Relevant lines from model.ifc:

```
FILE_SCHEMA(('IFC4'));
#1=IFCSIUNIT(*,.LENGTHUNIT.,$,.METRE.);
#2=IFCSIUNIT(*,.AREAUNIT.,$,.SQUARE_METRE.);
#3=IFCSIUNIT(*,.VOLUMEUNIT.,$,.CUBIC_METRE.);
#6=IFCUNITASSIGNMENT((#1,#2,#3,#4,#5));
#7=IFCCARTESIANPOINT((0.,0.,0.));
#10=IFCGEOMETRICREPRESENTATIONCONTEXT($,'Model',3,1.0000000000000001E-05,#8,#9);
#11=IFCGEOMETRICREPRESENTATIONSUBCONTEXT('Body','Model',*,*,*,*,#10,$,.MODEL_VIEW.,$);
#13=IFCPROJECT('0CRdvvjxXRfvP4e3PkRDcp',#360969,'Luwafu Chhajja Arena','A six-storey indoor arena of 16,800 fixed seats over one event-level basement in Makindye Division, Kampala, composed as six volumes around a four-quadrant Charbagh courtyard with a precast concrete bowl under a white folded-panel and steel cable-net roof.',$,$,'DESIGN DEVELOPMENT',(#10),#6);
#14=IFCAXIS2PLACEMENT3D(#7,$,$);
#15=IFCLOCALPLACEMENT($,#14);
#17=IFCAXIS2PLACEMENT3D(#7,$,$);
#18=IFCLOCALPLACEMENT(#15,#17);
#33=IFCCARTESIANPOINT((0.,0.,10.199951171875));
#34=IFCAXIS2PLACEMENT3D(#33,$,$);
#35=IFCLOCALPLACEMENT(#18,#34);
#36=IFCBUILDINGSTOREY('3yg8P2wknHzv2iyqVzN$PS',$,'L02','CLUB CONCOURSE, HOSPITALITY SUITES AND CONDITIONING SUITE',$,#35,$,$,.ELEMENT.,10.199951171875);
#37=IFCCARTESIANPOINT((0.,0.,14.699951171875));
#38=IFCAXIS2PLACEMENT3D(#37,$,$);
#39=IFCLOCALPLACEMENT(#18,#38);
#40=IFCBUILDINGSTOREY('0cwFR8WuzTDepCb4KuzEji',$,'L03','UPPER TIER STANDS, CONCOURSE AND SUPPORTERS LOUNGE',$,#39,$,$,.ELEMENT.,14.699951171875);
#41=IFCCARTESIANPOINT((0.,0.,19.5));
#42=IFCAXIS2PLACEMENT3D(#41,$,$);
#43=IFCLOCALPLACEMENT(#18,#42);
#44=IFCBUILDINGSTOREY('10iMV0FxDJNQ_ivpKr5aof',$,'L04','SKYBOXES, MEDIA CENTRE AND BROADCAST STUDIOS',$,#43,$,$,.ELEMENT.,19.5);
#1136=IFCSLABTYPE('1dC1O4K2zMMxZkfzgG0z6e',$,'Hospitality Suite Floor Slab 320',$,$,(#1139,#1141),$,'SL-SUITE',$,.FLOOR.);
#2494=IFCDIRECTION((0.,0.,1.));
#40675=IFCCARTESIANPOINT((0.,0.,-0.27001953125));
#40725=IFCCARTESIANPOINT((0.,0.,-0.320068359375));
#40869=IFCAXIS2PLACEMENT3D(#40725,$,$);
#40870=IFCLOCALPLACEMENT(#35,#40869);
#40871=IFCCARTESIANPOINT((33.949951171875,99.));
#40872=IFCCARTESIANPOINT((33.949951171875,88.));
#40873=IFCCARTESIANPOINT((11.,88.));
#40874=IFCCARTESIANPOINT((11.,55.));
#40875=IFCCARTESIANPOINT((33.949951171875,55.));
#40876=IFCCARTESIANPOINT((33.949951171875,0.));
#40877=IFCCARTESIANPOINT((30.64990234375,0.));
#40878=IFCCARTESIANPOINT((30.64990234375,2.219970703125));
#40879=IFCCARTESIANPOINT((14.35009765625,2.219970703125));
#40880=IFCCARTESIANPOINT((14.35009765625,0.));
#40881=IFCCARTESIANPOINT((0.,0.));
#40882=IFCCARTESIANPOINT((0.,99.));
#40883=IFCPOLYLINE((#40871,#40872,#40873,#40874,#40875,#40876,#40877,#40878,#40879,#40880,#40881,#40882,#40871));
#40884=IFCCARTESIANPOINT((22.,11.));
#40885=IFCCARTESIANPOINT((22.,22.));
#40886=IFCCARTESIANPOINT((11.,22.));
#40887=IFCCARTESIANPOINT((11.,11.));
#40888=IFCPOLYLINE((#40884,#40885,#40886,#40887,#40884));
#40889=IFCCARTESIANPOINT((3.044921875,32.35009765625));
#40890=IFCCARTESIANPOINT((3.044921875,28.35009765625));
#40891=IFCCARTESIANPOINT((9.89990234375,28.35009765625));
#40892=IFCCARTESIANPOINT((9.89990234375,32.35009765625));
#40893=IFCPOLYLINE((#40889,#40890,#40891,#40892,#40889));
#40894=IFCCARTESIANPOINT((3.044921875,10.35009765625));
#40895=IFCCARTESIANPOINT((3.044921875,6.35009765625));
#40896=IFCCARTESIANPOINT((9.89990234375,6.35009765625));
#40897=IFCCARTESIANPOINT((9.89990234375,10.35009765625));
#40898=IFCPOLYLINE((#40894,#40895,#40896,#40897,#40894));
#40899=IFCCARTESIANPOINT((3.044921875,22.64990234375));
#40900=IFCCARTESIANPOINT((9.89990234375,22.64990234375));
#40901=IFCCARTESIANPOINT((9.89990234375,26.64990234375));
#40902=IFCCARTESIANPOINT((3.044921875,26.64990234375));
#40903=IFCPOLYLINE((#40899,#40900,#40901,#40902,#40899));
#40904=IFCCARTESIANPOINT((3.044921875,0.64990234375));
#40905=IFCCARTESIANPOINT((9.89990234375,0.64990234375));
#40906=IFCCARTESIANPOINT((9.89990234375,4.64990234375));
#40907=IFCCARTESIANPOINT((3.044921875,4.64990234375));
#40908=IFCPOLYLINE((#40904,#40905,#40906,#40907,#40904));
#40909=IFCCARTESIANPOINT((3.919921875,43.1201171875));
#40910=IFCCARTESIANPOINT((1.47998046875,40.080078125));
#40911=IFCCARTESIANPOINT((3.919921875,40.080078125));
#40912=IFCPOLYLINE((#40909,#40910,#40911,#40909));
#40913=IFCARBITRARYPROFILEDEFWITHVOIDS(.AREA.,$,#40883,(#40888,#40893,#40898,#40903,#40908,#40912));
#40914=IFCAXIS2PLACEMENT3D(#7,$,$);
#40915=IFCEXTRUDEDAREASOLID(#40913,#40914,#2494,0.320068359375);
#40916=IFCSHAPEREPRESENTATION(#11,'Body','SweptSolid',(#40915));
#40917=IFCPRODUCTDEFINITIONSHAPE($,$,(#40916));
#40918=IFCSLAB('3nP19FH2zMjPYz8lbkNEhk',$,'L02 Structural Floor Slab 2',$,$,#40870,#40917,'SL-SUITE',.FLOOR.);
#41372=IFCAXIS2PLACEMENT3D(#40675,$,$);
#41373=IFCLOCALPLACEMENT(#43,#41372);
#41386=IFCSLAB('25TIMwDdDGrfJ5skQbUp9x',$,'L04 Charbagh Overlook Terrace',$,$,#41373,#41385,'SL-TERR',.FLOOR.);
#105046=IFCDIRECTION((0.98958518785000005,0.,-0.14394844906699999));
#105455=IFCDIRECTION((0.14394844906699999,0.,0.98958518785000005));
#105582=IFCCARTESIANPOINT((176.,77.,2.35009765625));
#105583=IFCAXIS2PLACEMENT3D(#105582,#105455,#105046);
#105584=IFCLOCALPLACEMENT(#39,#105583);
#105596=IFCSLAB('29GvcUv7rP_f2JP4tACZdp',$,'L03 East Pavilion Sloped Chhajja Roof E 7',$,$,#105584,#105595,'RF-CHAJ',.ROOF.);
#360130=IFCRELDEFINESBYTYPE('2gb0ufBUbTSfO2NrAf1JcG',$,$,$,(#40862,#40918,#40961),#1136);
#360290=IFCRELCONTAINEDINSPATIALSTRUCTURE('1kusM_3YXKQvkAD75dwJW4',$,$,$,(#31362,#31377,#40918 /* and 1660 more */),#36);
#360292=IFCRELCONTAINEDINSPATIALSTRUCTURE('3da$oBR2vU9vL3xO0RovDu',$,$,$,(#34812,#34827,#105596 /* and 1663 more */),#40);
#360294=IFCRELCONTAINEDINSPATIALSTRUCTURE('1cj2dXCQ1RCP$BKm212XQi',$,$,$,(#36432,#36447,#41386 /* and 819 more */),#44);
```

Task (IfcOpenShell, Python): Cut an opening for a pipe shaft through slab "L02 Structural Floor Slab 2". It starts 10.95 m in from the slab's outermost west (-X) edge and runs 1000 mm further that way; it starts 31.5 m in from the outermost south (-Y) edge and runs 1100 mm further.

```python
import numpy as np
import ifcopenshell
import ifcopenshell.api.feature
import ifcopenshell.api.geometry
import ifcopenshell.api.root
import ifcopenshell.geom
import ifcopenshell.util.placement
import ifcopenshell.util.representation
import ifcopenshell.util.shape
import ifcopenshell.util.unit

model = ifcopenshell.open("model.ifc")
unit_scale = ifcopenshell.util.unit.calculate_unit_scale(model)
settings = ifcopenshell.geom.settings()


def volume(element):
    """Net volume in cubic metres, openings subtracted."""
    shape = ifcopenshell.geom.create_shape(settings, element)
    return ifcopenshell.util.shape.get_volume(shape.geometry)


slab = model.by_guid("3nP19FH2zMjPYz8lbkNEhk")
before = volume(slab)

# Extent in the slab's own axes, in metres. The edges named are its -X and -Y sides.
slab_shape = ifcopenshell.geom.create_shape(settings, slab)
vertices = ifcopenshell.util.shape.get_vertices(slab_shape.geometry)
x_min, y_min, bottom = vertices.min(axis=0)
top = vertices[:, 2].max()

opening = ifcopenshell.api.root.create_entity(model, ifc_class="IfcOpeningElement", name="Pipe shaft opening", predefined_type="OPENING")
context = ifcopenshell.util.representation.get_context(model, "Model", "Body", "MODEL_VIEW")
width, depth = 1, 1.1
outline = [(0.0, 0.0), (width, 0.0), (width, depth), (0.0, depth), (0.0, 0.0)]
# Overshoot both faces by 50 mm so the cut is clean.
shape = ifcopenshell.api.geometry.add_slab_representation(
    model, context=context, depth=top - bottom + 0.1, polyline=outline
)
ifcopenshell.api.geometry.assign_representation(model, product=opening, representation=shape)

matrix = ifcopenshell.util.placement.get_local_placement(slab.ObjectPlacement)
matrix[:, 3] = matrix @ np.append(np.array([x_min + 10.95, y_min + 31.5, bottom - 0.05]) / unit_scale, 1.0)
ifcopenshell.api.geometry.edit_object_placement(model, product=opening, matrix=matrix, is_si=False)
ifcopenshell.api.feature.add_feature(model, feature=opening, element=slab)

after = volume(slab)

print(f"slab volume {before:.3f} -> {after:.3f} m3")

model.write("model_edited.ifc")
```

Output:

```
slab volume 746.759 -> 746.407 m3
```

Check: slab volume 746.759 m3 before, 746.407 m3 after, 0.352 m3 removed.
